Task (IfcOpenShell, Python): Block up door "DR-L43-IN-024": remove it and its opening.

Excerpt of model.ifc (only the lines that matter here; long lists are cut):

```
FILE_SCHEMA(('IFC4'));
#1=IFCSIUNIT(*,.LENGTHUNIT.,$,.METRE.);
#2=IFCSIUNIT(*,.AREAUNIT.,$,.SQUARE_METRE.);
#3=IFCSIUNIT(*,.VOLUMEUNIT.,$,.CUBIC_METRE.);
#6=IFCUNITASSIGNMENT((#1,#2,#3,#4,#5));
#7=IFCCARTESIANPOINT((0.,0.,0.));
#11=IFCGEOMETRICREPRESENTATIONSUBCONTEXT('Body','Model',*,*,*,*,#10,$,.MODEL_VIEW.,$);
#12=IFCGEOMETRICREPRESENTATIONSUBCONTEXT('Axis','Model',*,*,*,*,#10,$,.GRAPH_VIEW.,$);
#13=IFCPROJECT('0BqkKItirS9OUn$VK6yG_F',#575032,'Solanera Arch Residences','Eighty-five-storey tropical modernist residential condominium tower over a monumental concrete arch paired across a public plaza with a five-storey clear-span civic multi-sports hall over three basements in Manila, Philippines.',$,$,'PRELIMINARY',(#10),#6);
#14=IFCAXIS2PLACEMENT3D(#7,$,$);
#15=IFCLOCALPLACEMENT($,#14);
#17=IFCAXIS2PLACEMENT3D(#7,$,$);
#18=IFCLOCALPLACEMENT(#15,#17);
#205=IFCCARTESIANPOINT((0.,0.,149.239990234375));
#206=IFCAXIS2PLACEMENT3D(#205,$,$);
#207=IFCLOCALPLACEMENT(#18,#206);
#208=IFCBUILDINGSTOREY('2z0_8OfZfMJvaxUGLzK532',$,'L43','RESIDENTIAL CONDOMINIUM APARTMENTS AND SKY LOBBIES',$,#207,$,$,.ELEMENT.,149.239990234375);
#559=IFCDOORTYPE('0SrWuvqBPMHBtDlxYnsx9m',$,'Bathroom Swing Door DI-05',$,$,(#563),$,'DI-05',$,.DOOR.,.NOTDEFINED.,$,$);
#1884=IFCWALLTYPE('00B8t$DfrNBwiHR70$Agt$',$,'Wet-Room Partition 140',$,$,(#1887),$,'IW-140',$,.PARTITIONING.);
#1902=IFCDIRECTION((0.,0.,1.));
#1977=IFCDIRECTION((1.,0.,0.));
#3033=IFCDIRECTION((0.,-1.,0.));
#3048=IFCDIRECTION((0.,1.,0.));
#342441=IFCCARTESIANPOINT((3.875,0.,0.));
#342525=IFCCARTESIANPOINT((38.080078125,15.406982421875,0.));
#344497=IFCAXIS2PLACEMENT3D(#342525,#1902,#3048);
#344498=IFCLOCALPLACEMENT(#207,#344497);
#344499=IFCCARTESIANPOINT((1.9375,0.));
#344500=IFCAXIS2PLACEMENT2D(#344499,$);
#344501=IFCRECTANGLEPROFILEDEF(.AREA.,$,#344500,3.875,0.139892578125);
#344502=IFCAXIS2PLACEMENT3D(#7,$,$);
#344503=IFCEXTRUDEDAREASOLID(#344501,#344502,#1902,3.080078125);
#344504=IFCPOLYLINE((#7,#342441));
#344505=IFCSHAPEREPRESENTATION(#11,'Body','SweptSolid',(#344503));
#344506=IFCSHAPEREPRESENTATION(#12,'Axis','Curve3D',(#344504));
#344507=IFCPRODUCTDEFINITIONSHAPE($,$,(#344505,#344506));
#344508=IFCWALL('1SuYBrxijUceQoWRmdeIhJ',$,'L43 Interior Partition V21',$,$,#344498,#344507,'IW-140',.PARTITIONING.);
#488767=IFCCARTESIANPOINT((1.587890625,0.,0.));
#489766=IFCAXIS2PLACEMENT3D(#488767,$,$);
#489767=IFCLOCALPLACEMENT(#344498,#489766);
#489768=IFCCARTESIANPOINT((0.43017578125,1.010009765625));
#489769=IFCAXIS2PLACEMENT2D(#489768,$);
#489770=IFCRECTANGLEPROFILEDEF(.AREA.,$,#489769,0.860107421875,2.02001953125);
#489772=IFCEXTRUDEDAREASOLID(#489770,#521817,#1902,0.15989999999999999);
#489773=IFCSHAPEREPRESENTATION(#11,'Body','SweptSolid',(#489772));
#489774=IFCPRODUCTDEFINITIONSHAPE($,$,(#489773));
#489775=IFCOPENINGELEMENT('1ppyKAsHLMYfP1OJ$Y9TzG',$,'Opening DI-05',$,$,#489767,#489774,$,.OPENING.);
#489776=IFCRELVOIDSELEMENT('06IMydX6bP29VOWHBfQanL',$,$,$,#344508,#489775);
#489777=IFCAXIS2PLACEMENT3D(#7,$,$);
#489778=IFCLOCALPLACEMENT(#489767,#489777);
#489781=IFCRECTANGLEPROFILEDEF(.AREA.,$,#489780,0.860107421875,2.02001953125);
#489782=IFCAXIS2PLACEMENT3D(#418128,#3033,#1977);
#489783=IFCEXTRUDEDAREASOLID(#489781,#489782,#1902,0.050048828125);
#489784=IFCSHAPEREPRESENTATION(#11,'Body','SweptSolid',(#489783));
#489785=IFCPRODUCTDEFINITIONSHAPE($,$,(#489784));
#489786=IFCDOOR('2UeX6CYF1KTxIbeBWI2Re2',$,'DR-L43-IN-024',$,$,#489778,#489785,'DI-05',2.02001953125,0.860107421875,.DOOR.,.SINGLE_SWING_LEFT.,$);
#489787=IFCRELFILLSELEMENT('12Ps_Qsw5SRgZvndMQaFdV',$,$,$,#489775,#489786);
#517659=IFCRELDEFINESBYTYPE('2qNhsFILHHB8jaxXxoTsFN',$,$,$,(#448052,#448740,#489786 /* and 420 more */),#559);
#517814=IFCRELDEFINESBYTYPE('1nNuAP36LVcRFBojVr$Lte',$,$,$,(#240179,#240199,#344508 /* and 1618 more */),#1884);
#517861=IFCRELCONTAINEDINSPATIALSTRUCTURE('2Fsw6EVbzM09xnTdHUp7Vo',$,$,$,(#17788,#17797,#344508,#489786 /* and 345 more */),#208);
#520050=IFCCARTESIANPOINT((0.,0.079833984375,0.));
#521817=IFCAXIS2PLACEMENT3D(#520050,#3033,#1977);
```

```python
import ifcopenshell
import ifcopenshell.api.feature
import ifcopenshell.api.root
import ifcopenshell.geom
import ifcopenshell.util.shape

model = ifcopenshell.open("model.ifc")
settings = ifcopenshell.geom.settings()


def volume(element):
    """Net volume in cubic metres, openings subtracted."""
    shape = ifcopenshell.geom.create_shape(settings, element)
    return ifcopenshell.util.shape.get_volume(shape.geometry)


door = model.by_guid("2UeX6CYF1KTxIbeBWI2Re2")
opening = door.FillsVoids[0].RelatingOpeningElement
wall = opening.VoidsElements[0].RelatingBuildingElement
before = volume(wall)

ifcopenshell.api.root.remove_product(model, product=door)
ifcopenshell.api.feature.remove_feature(model, feature=opening)

after = volume(wall)

print(f"wall volume {before:.3f} -> {after:.3f} m3")

model.write("model_edited.ifc")
```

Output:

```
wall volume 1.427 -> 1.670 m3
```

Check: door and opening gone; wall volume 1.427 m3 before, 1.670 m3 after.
